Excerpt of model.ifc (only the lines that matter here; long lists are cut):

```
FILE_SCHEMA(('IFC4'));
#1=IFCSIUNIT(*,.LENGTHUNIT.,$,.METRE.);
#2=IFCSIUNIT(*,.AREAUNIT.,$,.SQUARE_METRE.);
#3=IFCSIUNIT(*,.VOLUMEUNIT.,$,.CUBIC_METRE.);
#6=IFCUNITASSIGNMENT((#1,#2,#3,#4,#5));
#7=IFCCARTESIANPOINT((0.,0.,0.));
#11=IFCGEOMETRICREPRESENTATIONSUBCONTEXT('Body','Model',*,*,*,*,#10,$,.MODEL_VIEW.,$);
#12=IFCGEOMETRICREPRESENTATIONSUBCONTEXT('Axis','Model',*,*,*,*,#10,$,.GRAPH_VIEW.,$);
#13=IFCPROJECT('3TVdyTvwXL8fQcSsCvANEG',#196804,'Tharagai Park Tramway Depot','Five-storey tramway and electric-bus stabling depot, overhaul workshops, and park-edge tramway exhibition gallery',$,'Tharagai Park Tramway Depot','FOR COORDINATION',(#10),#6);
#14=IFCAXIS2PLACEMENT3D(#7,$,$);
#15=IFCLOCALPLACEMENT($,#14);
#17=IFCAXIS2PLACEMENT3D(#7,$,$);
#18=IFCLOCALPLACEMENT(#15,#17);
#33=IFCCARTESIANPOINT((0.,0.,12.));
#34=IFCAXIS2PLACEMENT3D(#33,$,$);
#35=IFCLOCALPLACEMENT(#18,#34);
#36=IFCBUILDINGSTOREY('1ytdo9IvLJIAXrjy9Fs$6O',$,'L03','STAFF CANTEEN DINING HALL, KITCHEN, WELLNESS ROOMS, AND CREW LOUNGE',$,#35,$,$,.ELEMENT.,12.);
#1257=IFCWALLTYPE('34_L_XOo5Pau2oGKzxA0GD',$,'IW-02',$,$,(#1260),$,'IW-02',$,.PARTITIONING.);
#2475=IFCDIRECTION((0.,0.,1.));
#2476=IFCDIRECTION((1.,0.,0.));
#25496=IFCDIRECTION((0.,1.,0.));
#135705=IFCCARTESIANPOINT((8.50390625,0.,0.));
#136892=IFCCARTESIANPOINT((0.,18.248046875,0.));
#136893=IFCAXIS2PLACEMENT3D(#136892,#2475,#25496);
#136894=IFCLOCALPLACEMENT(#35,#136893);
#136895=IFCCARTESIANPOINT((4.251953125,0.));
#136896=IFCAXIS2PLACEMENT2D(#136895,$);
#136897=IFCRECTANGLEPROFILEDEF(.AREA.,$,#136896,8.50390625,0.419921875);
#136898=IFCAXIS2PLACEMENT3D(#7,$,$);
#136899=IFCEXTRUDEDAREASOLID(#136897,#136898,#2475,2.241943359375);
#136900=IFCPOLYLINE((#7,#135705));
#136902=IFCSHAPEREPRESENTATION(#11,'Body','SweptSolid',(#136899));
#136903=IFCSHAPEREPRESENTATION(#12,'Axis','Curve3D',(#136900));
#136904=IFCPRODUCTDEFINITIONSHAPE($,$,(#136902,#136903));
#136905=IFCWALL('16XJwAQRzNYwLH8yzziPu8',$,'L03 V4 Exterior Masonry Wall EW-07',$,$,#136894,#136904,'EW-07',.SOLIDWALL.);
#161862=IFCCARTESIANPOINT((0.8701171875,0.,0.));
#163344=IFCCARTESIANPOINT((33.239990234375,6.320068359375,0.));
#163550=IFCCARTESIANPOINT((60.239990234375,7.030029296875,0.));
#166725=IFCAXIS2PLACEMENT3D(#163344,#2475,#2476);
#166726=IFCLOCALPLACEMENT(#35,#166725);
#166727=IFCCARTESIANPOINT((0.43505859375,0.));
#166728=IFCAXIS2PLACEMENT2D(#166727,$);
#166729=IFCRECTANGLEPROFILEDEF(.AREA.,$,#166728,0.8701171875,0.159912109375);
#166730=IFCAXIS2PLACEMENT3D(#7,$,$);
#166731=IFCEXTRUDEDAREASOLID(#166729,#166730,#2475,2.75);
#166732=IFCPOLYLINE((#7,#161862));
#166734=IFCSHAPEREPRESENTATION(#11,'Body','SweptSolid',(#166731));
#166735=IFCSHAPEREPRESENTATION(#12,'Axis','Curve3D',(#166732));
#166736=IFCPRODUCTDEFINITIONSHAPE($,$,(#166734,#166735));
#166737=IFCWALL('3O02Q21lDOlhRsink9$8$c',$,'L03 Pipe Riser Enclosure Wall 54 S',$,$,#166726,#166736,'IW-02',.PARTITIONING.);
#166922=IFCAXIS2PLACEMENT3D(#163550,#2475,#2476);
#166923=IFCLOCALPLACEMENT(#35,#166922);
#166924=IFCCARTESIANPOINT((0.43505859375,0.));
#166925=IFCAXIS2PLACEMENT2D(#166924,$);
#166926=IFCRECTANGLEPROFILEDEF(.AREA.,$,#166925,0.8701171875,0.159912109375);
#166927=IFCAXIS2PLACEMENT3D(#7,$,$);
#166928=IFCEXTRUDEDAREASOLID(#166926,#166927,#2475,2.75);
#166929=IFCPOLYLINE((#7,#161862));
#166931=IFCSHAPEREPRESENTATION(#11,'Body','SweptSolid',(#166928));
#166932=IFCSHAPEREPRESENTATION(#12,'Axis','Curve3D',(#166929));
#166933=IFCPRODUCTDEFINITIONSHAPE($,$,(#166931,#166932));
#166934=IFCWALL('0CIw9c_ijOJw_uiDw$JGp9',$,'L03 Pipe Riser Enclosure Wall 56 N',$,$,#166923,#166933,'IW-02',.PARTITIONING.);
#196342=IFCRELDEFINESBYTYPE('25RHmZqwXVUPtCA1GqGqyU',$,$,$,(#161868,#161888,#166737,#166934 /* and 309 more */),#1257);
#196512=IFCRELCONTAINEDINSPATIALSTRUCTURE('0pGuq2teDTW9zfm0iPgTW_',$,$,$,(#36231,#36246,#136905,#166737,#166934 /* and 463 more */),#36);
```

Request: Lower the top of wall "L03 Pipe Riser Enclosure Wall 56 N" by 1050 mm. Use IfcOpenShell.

```python
import ifcopenshell
import ifcopenshell.geom
import ifcopenshell.util.representation
import ifcopenshell.util.shape

model = ifcopenshell.open("model.ifc")
settings = ifcopenshell.geom.settings()


def volume(element):
    """Net volume in cubic metres, openings subtracted."""
    shape = ifcopenshell.geom.create_shape(settings, element)
    return ifcopenshell.util.shape.get_volume(shape.geometry)


wall = model.by_guid("0CIw9c_ijOJw_uiDw$JGp9")
before = volume(wall)

body = ifcopenshell.util.representation.get_representation(wall, "Model", "Body")
solid = body.Items[0]
old_height = solid.Depth
solid.Depth -= 1.05
after = volume(wall)

print(f"height {old_height:g} -> {solid.Depth:g}, volume {before:.3f} -> {after:.3f} m3")

model.write("model_v2.ifc")
```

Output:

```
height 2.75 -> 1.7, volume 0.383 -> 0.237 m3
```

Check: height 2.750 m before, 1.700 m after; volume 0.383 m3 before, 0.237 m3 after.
